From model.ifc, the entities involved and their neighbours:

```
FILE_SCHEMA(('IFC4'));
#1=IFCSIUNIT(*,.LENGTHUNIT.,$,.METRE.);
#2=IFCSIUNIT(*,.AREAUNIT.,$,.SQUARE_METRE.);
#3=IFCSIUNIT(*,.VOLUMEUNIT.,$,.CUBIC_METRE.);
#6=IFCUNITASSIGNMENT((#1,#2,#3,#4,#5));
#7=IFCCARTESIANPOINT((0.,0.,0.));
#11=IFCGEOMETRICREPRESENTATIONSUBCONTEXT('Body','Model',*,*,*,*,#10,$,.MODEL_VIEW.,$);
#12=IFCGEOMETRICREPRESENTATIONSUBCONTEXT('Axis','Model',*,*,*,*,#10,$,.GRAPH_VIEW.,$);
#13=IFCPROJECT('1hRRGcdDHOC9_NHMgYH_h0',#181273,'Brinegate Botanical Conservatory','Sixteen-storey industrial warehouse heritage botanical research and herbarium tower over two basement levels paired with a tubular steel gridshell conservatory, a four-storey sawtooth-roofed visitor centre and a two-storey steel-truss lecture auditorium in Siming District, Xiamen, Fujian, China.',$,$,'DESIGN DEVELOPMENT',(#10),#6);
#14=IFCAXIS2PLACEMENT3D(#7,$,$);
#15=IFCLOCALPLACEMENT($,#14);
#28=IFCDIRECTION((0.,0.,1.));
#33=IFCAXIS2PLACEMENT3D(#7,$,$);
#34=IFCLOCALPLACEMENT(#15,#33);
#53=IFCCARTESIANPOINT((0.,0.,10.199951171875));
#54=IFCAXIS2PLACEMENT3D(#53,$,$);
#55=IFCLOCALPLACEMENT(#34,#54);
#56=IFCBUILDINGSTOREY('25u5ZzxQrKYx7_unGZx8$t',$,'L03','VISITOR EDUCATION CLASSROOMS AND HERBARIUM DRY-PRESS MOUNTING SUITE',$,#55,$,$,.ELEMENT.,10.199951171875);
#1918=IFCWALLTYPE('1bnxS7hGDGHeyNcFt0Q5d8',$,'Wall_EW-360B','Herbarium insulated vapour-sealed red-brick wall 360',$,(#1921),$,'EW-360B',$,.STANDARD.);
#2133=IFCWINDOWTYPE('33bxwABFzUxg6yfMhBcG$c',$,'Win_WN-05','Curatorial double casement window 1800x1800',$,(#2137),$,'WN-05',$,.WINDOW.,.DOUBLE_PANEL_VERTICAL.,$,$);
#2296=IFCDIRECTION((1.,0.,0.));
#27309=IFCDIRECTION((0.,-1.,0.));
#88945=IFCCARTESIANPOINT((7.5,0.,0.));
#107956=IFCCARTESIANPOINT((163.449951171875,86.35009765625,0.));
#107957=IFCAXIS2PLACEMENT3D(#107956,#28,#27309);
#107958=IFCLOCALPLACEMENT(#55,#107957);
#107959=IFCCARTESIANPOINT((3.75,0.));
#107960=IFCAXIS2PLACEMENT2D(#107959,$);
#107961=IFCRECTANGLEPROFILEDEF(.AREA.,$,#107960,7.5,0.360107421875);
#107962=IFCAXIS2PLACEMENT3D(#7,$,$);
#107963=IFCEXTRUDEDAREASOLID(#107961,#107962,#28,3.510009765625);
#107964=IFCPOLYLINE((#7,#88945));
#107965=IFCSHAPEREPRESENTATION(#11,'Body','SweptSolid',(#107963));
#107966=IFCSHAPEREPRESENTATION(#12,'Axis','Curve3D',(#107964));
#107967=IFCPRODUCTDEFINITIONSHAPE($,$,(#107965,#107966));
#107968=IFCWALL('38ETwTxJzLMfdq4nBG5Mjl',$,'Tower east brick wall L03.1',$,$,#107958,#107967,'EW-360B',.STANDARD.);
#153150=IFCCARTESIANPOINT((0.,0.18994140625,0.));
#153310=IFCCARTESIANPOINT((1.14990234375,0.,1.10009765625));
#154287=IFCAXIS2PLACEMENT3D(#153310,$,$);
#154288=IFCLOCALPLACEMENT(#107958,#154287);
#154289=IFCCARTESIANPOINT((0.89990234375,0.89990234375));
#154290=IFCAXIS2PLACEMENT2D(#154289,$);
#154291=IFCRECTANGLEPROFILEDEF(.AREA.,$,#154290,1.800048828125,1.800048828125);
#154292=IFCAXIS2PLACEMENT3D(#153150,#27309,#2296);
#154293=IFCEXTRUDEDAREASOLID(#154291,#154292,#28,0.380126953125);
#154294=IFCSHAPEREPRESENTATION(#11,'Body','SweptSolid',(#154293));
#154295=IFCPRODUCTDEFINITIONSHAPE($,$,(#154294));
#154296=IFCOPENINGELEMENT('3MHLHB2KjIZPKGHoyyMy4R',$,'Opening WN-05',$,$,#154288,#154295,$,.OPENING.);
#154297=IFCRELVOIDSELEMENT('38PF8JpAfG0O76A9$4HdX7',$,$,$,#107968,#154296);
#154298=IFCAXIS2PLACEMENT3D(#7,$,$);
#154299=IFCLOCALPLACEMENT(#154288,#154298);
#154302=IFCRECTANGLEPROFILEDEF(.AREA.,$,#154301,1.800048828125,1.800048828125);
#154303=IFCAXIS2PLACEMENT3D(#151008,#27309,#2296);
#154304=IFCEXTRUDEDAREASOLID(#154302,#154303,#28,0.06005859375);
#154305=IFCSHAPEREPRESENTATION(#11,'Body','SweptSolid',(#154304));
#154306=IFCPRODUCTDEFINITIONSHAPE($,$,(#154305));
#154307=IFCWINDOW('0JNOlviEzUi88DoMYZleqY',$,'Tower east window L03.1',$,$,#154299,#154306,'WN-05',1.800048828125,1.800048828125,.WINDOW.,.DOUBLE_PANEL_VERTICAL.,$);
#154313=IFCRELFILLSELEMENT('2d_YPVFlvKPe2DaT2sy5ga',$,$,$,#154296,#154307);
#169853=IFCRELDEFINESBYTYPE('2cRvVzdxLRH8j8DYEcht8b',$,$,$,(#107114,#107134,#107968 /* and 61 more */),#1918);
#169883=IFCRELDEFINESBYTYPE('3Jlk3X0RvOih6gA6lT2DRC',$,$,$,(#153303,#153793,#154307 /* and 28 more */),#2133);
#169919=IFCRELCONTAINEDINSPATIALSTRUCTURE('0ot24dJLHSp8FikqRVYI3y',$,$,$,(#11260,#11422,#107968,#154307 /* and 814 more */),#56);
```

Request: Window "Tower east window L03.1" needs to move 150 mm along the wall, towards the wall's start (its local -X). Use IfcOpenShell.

```python
import ifcopenshell
import ifcopenshell.api.geometry
import ifcopenshell.util.placement

model = ifcopenshell.open("model.ifc")

window = model.by_id(154307)
opening = window.FillsVoids[0].RelatingOpeningElement
wall = opening.VoidsElements[0].RelatingBuildingElement

wall_matrix = ifcopenshell.util.placement.get_local_placement(wall.ObjectPlacement)
shift = wall_matrix[:3, 0] * -0.15
before = ifcopenshell.util.placement.get_local_placement(window.ObjectPlacement)[:3, 3].copy()

# The window is placed relative to its opening, so it follows when the opening moves.
matrix = ifcopenshell.util.placement.get_local_placement(opening.ObjectPlacement)
matrix[:3, 3] += shift
ifcopenshell.api.geometry.edit_object_placement(
    model, product=opening, matrix=matrix, is_si=False, should_transform_children=True
)

after = ifcopenshell.util.placement.get_local_placement(window.ObjectPlacement)[:3, 3]
print("window moved by", (after - before).round(3) + 0.0)

model.write("model_edited.ifc")
```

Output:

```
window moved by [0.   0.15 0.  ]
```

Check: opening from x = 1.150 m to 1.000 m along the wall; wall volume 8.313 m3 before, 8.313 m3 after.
